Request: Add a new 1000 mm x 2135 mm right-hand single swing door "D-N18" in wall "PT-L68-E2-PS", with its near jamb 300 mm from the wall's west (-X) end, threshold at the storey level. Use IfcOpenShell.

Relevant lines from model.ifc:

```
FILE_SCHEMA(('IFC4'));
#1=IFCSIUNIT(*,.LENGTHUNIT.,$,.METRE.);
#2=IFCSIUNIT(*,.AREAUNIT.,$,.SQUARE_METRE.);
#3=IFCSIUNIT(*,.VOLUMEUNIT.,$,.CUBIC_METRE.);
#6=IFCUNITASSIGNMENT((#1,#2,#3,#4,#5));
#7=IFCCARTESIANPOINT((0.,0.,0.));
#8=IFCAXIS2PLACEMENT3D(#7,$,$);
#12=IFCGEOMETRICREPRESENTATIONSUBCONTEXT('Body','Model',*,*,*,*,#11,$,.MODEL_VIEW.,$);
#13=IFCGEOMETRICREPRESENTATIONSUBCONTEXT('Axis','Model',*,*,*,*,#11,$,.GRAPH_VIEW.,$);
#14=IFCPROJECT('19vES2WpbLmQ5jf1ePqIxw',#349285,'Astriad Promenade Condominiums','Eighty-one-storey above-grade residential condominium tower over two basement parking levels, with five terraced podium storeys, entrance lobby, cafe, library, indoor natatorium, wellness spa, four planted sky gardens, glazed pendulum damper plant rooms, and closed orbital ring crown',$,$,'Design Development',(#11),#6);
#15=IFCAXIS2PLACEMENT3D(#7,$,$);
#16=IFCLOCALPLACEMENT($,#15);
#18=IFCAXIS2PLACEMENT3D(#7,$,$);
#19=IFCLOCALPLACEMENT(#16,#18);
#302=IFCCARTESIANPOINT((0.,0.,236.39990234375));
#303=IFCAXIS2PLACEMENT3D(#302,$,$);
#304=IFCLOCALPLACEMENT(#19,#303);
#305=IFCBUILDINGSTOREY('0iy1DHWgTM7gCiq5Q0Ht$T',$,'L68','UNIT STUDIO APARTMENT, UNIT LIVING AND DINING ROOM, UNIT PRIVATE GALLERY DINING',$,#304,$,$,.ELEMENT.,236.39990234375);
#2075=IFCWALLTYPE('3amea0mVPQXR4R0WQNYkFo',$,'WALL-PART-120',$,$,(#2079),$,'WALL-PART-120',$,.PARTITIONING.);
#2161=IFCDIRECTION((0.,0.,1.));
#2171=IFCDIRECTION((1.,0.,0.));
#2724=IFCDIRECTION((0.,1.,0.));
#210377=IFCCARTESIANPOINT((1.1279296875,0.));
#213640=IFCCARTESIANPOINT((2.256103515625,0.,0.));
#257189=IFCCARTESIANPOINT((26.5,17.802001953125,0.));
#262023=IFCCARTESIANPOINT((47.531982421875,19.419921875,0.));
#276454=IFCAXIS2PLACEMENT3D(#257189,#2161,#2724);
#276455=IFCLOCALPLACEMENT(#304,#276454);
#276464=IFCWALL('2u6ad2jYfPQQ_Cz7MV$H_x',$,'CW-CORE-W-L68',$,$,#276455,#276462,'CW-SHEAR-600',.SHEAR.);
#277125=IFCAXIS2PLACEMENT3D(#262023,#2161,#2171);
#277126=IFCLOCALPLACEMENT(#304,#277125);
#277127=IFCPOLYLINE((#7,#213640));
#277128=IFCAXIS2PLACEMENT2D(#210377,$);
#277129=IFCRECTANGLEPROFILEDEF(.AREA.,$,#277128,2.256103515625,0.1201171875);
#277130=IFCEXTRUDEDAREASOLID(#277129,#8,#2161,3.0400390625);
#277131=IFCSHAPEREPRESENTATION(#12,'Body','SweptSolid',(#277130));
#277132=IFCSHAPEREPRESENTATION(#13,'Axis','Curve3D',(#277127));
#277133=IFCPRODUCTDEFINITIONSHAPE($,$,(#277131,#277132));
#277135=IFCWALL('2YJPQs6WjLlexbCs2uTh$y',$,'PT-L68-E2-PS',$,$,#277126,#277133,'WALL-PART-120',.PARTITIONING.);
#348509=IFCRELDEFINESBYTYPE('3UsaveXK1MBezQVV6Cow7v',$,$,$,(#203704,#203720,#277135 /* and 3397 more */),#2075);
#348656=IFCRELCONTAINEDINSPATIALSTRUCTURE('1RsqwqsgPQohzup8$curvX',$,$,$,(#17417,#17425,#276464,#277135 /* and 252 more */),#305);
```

```python
import numpy as np
import ifcopenshell
import ifcopenshell.api.feature
import ifcopenshell.api.geometry
import ifcopenshell.api.root
import ifcopenshell.api.spatial
import ifcopenshell.geom
import ifcopenshell.util.element
import ifcopenshell.util.placement
import ifcopenshell.util.representation
import ifcopenshell.util.shape
import ifcopenshell.util.unit

model = ifcopenshell.open("model.ifc")
unit_scale = ifcopenshell.util.unit.calculate_unit_scale(model)
settings = ifcopenshell.geom.settings()


def volume(element):
    """Net volume in cubic metres, openings subtracted."""
    shape = ifcopenshell.geom.create_shape(settings, element)
    return ifcopenshell.util.shape.get_volume(shape.geometry)


wall = model.by_guid("2YJPQs6WjLlexbCs2uTh$y")
storey = ifcopenshell.util.element.get_container(wall, ifc_class="IfcBuildingStorey")
context = ifcopenshell.util.representation.get_context(model, "Model", "Body", "MODEL_VIEW")
before = volume(wall)

width, height, from_end, sill = 1, 2.135, 0.3, 0.0  # metres

# The wall runs along its own X axis, and the end named is its -X end.
wall_shape = ifcopenshell.geom.create_shape(settings, wall)
x, y, z = ifcopenshell.util.shape.get_vertices(wall_shape.geometry).T
start = x.min() + from_end
face, thickness = float(y.min()), float(y.max() - y.min())
wall_matrix = ifcopenshell.util.placement.get_local_placement(wall.ObjectPlacement)
level = ifcopenshell.util.placement.get_local_placement(storey.ObjectPlacement)[2, 3]


def in_wall(x, y):
    """Placement at x, y metres in the wall's axes, at sill height."""
    matrix = wall_matrix.copy()
    matrix[:, 3] = wall_matrix @ np.array([x / unit_scale, y / unit_scale, 0.0, 1.0])
    matrix[2, 3] = level + sill / unit_scale
    return matrix


# Opening: a box that overshoots both wall faces by 50 mm.
opening = ifcopenshell.api.root.create_entity(model, ifc_class="IfcOpeningElement", predefined_type="OPENING")
box = ifcopenshell.api.geometry.add_wall_representation(
    model, context=context, length=width, height=height, thickness=thickness + 0.1
)
ifcopenshell.api.geometry.assign_representation(model, product=opening, representation=box)
ifcopenshell.api.geometry.edit_object_placement(model, product=opening, matrix=in_wall(start, face - 0.05), is_si=False)
ifcopenshell.api.feature.add_feature(model, feature=opening, element=wall)

door = ifcopenshell.api.root.create_entity(model, ifc_class="IfcDoor", name="D-N18", predefined_type="DOOR")
door.OverallWidth, door.OverallHeight = width / unit_scale, height / unit_scale
door.OperationType = "SINGLE_SWING_RIGHT"
body = ifcopenshell.api.geometry.add_door_representation(
    model,
    context=context,
    overall_width=door.OverallWidth,
    overall_height=door.OverallHeight,
    operation_type="SINGLE_SWING_RIGHT",
    lining_properties={"LiningDepth": thickness / unit_scale, "ThresholdDepth": thickness / unit_scale},
)
ifcopenshell.api.geometry.assign_representation(model, product=door, representation=body)
ifcopenshell.api.spatial.assign_container(model, products=[door], relating_structure=storey)
ifcopenshell.api.feature.add_filling(model, opening=opening, element=door)

# The lining spans the wall, so the door starts at the wall face.
ifcopenshell.api.geometry.edit_object_placement(model, product=door, matrix=in_wall(start, face), is_si=False)

after = volume(wall)

print(f"wall volume {before:.3f} -> {after:.3f} m3")

model.write("model_edited.ifc")
```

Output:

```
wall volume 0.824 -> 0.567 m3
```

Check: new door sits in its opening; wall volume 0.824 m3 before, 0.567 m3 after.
